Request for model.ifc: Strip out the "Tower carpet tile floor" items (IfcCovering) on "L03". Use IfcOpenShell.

First a look at what the model holds.

```python
import ifcopenshell
import ifcopenshell.util.element

model = ifcopenshell.open("model.ifc")
print(model.schema)
storey = next(s for s in model.by_type("IfcBuildingStorey") if s.Name == "L03")
coverings = [e for e in ifcopenshell.util.element.get_decomposition(storey) if e.is_a("IfcCovering")]
seen = {}
for e in coverings:
    element_type = ifcopenshell.util.element.get_type(e)
    name = element_type.Name if element_type not in (None, e) else None
    seen[name] = seen.get(name, 0) + 1
for name, count in sorted(seen.items(), key=str):
    print(count, "x", name)
```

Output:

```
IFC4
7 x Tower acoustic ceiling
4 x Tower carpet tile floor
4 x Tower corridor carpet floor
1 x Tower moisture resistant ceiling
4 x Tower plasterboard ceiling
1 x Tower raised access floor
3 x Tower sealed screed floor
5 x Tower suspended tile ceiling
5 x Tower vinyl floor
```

```python
import ifcopenshell
import ifcopenshell.api.root
import ifcopenshell.util.element

model = ifcopenshell.open("model.ifc")

storey = next(s for s in model.by_type("IfcBuildingStorey") if s.Name == "L03")
coverings = [e for e in ifcopenshell.util.element.get_decomposition(storey) if e.is_a("IfcCovering")]
targets = [e for e in coverings if (t := ifcopenshell.util.element.get_type(e)) not in (None, e) and t.Name == "Tower carpet tile floor"]

for e in targets:
    ifcopenshell.api.root.remove_product(model, product=e)
print(len(targets), "removed")

model.write("model_updated.ifc")
```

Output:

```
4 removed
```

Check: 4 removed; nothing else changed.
